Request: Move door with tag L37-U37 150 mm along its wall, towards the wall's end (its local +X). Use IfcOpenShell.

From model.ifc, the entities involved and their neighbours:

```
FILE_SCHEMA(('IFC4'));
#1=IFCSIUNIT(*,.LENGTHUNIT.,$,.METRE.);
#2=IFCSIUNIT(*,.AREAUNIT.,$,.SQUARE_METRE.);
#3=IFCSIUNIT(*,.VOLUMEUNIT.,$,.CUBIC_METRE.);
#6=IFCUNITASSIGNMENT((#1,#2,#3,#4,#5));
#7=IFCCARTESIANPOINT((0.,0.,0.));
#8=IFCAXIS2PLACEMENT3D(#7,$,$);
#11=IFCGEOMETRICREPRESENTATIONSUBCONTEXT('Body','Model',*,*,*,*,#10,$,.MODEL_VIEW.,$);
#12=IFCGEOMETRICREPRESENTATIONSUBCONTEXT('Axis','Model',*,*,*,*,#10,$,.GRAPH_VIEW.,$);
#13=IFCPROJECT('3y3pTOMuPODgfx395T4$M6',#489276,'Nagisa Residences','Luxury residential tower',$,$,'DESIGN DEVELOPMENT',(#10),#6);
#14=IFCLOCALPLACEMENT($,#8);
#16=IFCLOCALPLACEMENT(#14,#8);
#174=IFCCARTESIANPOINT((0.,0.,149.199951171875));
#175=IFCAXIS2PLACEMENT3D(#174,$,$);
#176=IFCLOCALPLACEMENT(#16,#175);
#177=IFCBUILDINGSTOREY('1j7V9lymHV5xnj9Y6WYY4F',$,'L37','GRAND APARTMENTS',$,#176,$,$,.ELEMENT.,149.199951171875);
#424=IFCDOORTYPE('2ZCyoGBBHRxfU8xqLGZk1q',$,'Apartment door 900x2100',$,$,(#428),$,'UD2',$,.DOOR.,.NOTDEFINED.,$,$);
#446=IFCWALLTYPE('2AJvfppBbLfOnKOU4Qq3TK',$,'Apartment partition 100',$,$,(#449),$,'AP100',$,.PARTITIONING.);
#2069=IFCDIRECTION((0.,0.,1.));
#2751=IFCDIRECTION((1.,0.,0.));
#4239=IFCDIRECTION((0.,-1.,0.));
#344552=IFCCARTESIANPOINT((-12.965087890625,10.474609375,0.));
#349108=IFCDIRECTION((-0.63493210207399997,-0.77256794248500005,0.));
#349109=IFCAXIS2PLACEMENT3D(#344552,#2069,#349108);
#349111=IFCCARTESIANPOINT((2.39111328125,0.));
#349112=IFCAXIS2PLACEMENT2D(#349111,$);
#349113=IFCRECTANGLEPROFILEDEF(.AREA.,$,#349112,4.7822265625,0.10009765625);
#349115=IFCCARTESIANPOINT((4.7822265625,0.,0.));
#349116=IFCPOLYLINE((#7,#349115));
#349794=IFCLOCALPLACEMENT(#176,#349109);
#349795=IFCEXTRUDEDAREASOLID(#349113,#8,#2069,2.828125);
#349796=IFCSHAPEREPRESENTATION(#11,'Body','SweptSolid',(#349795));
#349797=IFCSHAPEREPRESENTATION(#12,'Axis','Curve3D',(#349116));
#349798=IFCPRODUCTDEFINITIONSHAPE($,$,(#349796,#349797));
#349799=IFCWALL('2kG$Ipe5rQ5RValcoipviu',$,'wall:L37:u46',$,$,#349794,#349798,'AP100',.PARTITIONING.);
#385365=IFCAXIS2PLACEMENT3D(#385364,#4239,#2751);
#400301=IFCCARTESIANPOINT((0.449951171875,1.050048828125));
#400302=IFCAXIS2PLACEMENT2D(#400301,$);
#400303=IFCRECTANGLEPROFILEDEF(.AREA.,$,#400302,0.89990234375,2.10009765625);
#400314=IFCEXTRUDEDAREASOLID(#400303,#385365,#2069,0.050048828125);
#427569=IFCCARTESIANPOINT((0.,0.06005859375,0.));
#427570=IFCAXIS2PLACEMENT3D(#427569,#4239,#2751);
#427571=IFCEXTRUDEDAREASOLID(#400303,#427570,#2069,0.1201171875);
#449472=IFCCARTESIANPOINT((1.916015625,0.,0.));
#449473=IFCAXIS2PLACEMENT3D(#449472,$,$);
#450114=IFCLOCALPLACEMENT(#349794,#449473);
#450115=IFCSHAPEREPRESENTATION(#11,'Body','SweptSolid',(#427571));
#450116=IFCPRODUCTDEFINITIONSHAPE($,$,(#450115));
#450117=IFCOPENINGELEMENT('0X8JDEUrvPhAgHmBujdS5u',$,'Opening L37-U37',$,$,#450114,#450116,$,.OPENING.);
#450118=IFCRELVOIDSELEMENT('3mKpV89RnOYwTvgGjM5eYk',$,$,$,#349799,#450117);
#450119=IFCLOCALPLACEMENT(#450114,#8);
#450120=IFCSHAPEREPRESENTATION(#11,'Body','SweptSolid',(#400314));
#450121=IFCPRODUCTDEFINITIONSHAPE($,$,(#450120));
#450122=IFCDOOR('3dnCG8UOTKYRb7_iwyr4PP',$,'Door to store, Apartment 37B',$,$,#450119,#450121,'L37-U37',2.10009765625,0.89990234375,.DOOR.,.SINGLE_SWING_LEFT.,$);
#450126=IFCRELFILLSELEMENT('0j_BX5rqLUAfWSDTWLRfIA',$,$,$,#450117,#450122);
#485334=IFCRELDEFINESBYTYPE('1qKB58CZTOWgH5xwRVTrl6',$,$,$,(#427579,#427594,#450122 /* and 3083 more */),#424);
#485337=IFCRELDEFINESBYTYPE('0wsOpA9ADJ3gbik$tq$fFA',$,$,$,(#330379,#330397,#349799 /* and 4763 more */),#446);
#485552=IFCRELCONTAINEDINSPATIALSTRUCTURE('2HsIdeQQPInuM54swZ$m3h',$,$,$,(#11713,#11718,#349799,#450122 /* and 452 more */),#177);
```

```python
import ifcopenshell
import ifcopenshell.api.geometry
import ifcopenshell.util.placement
import ifcopenshell.util.unit

model = ifcopenshell.open("model.ifc")
unit_scale = ifcopenshell.util.unit.calculate_unit_scale(model)

door = model.by_guid("3dnCG8UOTKYRb7_iwyr4PP")
opening = door.FillsVoids[0].RelatingOpeningElement
wall = opening.VoidsElements[0].RelatingBuildingElement

wall_matrix = ifcopenshell.util.placement.get_local_placement(wall.ObjectPlacement)
shift = wall_matrix[:3, 0] * 0.15 / unit_scale
before = ifcopenshell.util.placement.get_local_placement(door.ObjectPlacement)[:3, 3].copy()

# The door is placed relative to its opening, so it follows when the opening moves.
matrix = ifcopenshell.util.placement.get_local_placement(opening.ObjectPlacement)
matrix[:3, 3] += shift
ifcopenshell.api.geometry.edit_object_placement(
    model, product=opening, matrix=matrix, is_si=False, should_transform_children=True
)

after = ifcopenshell.util.placement.get_local_placement(door.ObjectPlacement)[:3, 3]
print("door moved by", (after - before).round(3) + 0.0)

model.write("model_edited.ifc")
```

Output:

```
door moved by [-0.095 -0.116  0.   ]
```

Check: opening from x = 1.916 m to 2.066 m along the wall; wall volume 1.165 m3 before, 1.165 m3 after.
